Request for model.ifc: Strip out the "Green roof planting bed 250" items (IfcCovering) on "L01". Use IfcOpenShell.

First a look at what the model holds.

```python
import ifcopenshell
import ifcopenshell.util.element

model = ifcopenshell.open("model.ifc")
print(model.schema)
storey = next(s for s in model.by_type("IfcBuildingStorey") if s.Name == "L01")
coverings = [e for e in ifcopenshell.util.element.get_decomposition(storey) if e.is_a("IfcCovering")]
seen = {}
for e in coverings:
    element_type = ifcopenshell.util.element.get_type(e)
    name = element_type.Name if element_type not in (None, e) else None
    seen[name] = seen.get(name, 0) + 1
for name, count in sorted(seen.items(), key=str):
    print(count, "x", name)
```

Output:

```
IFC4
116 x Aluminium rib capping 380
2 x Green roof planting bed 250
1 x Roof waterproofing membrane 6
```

```python
import ifcopenshell
import ifcopenshell.api.root
import ifcopenshell.util.element

model = ifcopenshell.open("model.ifc")

storey = next(s for s in model.by_type("IfcBuildingStorey") if s.Name == "L01")
coverings = [e for e in ifcopenshell.util.element.get_decomposition(storey) if e.is_a("IfcCovering")]
targets = [e for e in coverings if (t := ifcopenshell.util.element.get_type(e)) not in (None, e) and t.Name == "Green roof planting bed 250"]

for e in targets:
    ifcopenshell.api.root.remove_product(model, product=e)
print(len(targets), "removed")

model.write("model_updated.ifc")
```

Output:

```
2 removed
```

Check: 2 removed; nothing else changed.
